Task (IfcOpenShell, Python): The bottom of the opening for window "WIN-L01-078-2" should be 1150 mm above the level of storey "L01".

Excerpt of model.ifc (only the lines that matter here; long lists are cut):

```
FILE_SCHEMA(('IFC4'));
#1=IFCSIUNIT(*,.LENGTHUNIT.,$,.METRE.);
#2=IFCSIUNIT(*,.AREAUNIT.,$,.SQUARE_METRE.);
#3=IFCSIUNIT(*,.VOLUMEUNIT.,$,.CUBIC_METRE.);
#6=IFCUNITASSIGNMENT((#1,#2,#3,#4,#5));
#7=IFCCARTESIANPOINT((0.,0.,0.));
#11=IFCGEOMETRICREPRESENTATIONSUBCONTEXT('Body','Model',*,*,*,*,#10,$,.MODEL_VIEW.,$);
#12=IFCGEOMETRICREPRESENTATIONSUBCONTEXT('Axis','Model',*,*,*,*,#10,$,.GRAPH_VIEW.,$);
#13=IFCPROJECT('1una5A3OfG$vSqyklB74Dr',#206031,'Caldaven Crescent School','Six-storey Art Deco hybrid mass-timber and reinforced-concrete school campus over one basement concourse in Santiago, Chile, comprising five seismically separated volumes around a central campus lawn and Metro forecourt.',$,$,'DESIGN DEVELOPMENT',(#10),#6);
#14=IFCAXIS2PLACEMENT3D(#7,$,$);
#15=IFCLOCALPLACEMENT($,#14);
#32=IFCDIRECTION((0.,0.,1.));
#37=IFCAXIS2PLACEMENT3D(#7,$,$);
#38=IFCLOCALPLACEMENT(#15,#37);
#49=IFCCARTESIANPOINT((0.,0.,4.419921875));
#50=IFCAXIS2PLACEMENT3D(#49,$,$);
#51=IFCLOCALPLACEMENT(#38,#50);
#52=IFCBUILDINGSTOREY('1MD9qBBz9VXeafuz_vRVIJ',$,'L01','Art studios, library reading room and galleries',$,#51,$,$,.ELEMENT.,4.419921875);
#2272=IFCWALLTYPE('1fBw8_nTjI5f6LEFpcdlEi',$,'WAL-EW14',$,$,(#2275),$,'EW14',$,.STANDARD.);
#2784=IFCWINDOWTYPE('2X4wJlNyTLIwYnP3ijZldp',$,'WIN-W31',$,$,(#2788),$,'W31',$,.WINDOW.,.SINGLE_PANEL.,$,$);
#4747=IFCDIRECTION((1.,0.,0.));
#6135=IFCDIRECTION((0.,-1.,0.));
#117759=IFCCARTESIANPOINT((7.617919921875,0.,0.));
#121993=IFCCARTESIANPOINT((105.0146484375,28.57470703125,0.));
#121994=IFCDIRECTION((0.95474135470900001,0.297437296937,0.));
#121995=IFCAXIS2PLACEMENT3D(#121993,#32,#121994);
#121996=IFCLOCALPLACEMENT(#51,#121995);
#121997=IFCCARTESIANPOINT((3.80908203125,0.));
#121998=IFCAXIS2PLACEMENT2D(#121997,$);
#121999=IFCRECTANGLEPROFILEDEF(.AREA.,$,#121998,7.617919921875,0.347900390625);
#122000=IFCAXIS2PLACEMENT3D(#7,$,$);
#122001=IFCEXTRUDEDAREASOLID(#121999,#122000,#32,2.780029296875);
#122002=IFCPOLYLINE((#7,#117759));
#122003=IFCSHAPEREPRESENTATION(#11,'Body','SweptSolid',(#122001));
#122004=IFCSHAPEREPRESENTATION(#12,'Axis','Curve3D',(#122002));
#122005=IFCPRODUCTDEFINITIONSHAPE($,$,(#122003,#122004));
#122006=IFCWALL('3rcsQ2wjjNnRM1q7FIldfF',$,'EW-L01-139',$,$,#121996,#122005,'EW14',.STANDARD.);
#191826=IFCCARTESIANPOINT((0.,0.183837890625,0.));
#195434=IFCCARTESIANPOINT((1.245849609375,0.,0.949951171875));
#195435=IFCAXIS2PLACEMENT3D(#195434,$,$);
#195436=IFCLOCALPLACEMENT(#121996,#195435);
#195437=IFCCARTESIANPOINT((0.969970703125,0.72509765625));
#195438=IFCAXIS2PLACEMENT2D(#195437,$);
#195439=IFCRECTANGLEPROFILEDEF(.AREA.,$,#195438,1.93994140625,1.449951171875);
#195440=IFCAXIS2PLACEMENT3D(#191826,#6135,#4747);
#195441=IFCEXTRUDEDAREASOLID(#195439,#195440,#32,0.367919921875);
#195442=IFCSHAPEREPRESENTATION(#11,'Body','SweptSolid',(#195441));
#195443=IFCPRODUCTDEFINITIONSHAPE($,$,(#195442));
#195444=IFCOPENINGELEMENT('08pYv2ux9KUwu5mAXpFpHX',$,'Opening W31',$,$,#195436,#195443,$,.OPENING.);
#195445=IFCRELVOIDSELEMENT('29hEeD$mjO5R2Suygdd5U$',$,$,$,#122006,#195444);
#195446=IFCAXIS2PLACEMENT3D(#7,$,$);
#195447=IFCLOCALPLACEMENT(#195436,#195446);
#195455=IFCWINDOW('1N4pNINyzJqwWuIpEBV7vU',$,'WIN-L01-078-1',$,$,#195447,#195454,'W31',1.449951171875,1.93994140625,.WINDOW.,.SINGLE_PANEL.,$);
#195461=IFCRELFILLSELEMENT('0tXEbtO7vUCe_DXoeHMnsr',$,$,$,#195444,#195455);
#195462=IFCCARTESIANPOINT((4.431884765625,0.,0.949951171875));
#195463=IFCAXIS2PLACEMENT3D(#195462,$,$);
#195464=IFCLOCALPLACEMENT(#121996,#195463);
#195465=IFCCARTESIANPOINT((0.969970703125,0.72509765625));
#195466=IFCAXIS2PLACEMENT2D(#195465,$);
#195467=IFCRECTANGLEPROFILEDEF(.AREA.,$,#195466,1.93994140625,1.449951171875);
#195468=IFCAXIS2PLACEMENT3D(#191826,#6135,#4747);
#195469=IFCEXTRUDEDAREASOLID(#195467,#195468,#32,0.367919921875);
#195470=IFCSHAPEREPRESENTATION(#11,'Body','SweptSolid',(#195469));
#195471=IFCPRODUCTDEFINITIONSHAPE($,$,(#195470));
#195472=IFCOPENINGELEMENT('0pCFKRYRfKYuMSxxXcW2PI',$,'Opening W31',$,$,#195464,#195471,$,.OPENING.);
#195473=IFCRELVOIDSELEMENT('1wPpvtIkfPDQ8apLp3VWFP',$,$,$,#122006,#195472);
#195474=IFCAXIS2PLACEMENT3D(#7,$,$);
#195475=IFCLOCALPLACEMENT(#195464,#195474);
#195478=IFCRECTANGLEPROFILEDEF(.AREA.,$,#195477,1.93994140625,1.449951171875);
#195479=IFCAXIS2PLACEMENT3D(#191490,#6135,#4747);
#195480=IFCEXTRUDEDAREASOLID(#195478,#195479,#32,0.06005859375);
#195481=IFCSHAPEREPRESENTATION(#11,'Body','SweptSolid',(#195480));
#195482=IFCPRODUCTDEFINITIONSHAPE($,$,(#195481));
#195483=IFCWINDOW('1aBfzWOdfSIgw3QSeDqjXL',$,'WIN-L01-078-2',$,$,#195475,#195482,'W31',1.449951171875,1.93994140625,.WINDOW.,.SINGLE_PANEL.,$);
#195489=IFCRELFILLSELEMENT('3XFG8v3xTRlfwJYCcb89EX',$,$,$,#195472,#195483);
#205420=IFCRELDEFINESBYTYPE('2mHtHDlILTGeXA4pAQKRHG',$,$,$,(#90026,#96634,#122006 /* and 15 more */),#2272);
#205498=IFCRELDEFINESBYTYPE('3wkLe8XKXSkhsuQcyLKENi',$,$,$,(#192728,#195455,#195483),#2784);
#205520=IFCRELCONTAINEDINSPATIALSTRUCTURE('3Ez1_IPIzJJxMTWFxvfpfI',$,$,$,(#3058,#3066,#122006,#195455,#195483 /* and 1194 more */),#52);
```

```python
import numpy as np
import ifcopenshell
import ifcopenshell.api.geometry
import ifcopenshell.geom
import ifcopenshell.util.element
import ifcopenshell.util.placement
import ifcopenshell.util.shape
import ifcopenshell.util.unit

model = ifcopenshell.open("model.ifc")
unit_scale = ifcopenshell.util.unit.calculate_unit_scale(model)

window = model.by_id(195483)
opening = window.FillsVoids[0].RelatingOpeningElement
storey = ifcopenshell.util.element.get_container(window, ifc_class="IfcBuildingStorey")
level = ifcopenshell.util.placement.get_local_placement(storey.ObjectPlacement)[2, 3]

# The opening's origin need not be at the sill, so measure its lowest point.
shape = ifcopenshell.geom.create_shape(ifcopenshell.geom.settings(), opening)
bottom = ifcopenshell.util.shape.get_shape_bottom_elevation(shape, shape.geometry) / unit_scale
dz = level + 1.15 / unit_scale - bottom

shift = np.array([0.0, 0.0, dz])
# The window is placed relative to its opening, so it follows when the opening moves.
matrix = ifcopenshell.util.placement.get_local_placement(opening.ObjectPlacement)
matrix[:3, 3] += shift
ifcopenshell.api.geometry.edit_object_placement(
    model, product=opening, matrix=matrix, is_si=False, should_transform_children=True
)

print(f"moved by {dz * unit_scale:+.3f} m")

model.write("model_rev.ifc")
```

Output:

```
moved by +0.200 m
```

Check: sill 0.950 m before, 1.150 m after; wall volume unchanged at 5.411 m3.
